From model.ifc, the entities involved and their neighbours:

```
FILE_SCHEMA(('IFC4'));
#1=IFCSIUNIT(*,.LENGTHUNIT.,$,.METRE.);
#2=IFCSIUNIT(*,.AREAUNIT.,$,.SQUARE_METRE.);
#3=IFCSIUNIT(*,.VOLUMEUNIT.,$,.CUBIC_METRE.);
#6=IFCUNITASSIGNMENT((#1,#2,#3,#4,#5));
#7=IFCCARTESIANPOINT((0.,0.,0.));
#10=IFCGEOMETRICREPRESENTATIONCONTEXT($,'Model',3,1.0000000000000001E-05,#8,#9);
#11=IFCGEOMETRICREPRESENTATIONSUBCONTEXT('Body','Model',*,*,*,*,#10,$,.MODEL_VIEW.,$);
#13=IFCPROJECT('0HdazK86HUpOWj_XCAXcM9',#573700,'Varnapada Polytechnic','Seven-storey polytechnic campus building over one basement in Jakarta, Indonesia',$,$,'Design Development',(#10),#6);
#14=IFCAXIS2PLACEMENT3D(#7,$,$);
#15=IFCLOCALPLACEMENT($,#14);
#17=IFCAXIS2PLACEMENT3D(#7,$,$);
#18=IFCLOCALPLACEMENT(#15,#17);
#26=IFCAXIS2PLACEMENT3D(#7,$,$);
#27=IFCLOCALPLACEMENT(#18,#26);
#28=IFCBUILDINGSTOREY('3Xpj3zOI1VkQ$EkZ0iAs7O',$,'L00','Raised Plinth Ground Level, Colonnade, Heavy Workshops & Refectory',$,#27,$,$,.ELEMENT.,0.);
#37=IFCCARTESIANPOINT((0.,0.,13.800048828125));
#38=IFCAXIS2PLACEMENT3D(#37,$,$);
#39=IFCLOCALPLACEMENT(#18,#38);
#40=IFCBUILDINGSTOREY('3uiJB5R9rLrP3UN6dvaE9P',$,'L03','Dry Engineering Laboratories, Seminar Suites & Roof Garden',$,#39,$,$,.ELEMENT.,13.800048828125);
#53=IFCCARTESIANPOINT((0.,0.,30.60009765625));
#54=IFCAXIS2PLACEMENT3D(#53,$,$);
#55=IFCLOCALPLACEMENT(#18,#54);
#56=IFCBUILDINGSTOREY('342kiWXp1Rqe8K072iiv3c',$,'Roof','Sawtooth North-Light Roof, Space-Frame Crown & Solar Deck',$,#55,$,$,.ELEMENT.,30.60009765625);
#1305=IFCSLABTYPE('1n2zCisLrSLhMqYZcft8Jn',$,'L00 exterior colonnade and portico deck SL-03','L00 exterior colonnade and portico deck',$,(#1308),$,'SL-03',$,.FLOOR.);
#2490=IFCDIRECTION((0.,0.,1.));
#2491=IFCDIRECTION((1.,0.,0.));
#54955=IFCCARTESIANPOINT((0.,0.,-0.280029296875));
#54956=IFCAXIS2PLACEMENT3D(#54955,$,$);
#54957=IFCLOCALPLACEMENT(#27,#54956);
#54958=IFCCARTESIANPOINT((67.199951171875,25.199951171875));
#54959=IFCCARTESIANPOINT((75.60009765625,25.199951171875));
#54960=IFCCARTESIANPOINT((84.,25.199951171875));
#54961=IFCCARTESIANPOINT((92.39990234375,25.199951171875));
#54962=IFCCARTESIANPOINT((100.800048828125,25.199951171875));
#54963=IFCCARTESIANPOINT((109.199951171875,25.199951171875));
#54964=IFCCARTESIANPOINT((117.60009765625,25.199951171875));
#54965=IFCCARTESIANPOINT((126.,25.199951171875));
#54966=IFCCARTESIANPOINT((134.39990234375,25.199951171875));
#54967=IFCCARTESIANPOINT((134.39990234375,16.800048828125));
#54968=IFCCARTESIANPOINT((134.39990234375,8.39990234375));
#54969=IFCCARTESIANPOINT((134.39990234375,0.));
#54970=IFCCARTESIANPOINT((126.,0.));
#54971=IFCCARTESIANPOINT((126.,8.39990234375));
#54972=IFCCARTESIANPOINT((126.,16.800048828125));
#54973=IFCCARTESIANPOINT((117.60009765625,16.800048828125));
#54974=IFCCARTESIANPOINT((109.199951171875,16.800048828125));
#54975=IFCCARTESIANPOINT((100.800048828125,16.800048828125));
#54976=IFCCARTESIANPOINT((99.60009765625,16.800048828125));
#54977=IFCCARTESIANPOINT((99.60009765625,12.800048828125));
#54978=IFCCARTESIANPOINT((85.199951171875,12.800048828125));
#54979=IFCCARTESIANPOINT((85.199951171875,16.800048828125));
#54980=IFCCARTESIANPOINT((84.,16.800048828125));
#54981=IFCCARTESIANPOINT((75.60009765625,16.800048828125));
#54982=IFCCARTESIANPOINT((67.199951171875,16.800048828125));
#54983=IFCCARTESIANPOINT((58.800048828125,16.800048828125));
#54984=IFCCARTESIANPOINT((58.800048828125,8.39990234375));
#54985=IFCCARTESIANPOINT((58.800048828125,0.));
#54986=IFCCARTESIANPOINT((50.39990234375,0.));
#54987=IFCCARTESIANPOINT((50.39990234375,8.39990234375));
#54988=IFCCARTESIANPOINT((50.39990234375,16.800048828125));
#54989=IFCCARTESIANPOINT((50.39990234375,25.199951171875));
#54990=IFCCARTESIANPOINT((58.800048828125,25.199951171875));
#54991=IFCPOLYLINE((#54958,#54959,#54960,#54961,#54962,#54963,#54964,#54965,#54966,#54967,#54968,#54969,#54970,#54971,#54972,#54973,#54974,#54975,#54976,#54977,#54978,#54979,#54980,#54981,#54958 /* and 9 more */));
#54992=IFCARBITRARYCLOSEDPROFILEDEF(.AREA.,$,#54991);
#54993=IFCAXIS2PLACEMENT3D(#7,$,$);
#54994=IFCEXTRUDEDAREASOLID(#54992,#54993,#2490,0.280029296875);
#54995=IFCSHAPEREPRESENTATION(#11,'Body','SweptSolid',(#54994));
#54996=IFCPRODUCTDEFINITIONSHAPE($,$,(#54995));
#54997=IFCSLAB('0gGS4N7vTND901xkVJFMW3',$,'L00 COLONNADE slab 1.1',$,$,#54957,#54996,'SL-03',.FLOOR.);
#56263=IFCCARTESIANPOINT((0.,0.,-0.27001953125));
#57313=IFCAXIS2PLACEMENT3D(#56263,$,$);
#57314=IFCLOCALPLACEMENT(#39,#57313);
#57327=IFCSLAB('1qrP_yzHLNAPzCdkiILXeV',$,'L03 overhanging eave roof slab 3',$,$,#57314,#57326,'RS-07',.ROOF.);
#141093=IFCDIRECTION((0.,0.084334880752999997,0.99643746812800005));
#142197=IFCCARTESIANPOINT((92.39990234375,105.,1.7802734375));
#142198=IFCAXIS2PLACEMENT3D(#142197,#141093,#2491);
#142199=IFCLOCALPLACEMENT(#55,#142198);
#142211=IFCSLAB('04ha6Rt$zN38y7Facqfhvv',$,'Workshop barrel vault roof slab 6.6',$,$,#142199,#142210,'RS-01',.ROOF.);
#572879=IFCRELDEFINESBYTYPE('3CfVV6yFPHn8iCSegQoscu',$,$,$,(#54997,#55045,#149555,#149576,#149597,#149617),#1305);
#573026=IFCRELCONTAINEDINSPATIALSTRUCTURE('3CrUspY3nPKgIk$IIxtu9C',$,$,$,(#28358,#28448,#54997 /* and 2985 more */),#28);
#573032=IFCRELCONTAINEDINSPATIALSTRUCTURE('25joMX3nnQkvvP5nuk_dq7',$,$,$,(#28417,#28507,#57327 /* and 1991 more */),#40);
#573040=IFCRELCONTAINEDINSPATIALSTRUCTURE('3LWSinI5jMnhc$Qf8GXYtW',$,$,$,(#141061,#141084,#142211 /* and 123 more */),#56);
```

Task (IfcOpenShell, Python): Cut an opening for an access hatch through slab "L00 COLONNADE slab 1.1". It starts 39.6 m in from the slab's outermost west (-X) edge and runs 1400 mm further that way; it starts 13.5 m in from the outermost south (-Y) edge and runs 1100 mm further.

```python
import numpy as np
import ifcopenshell
import ifcopenshell.api.feature
import ifcopenshell.api.geometry
import ifcopenshell.api.root
import ifcopenshell.geom
import ifcopenshell.util.placement
import ifcopenshell.util.representation
import ifcopenshell.util.shape
import ifcopenshell.util.unit

model = ifcopenshell.open("model.ifc")
unit_scale = ifcopenshell.util.unit.calculate_unit_scale(model)
settings = ifcopenshell.geom.settings()


def volume(element):
    """Net volume in cubic metres, openings subtracted."""
    shape = ifcopenshell.geom.create_shape(settings, element)
    return ifcopenshell.util.shape.get_volume(shape.geometry)


slab = model.by_guid("0gGS4N7vTND901xkVJFMW3")
before = volume(slab)

# Extent in the slab's own axes, in metres. The edges named are its -X and -Y sides.
slab_shape = ifcopenshell.geom.create_shape(settings, slab)
vertices = ifcopenshell.util.shape.get_vertices(slab_shape.geometry)
x_min, y_min, bottom = vertices.min(axis=0)
top = vertices[:, 2].max()

opening = ifcopenshell.api.root.create_entity(model, ifc_class="IfcOpeningElement", name="Access hatch opening", predefined_type="OPENING")
context = ifcopenshell.util.representation.get_context(model, "Model", "Body", "MODEL_VIEW")
width, depth = 1.4, 1.1
outline = [(0.0, 0.0), (width, 0.0), (width, depth), (0.0, depth), (0.0, 0.0)]
# Overshoot both faces by 50 mm so the cut is clean.
shape = ifcopenshell.api.geometry.add_slab_representation(
    model, context=context, depth=top - bottom + 0.1, polyline=outline
)
ifcopenshell.api.geometry.assign_representation(model, product=opening, representation=shape)

matrix = ifcopenshell.util.placement.get_local_placement(slab.ObjectPlacement)
matrix[:, 3] = matrix @ np.append(np.array([x_min + 39.6, y_min + 13.5, bottom - 0.05]) / unit_scale, 1.0)
ifcopenshell.api.geometry.edit_object_placement(model, product=opening, matrix=matrix, is_si=False)
ifcopenshell.api.feature.add_feature(model, feature=opening, element=slab)

after = volume(slab)

print(f"slab volume {before:.3f} -> {after:.3f} m3")

model.write("model_v2.ifc")
```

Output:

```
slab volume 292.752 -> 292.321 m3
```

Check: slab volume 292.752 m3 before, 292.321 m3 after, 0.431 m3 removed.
